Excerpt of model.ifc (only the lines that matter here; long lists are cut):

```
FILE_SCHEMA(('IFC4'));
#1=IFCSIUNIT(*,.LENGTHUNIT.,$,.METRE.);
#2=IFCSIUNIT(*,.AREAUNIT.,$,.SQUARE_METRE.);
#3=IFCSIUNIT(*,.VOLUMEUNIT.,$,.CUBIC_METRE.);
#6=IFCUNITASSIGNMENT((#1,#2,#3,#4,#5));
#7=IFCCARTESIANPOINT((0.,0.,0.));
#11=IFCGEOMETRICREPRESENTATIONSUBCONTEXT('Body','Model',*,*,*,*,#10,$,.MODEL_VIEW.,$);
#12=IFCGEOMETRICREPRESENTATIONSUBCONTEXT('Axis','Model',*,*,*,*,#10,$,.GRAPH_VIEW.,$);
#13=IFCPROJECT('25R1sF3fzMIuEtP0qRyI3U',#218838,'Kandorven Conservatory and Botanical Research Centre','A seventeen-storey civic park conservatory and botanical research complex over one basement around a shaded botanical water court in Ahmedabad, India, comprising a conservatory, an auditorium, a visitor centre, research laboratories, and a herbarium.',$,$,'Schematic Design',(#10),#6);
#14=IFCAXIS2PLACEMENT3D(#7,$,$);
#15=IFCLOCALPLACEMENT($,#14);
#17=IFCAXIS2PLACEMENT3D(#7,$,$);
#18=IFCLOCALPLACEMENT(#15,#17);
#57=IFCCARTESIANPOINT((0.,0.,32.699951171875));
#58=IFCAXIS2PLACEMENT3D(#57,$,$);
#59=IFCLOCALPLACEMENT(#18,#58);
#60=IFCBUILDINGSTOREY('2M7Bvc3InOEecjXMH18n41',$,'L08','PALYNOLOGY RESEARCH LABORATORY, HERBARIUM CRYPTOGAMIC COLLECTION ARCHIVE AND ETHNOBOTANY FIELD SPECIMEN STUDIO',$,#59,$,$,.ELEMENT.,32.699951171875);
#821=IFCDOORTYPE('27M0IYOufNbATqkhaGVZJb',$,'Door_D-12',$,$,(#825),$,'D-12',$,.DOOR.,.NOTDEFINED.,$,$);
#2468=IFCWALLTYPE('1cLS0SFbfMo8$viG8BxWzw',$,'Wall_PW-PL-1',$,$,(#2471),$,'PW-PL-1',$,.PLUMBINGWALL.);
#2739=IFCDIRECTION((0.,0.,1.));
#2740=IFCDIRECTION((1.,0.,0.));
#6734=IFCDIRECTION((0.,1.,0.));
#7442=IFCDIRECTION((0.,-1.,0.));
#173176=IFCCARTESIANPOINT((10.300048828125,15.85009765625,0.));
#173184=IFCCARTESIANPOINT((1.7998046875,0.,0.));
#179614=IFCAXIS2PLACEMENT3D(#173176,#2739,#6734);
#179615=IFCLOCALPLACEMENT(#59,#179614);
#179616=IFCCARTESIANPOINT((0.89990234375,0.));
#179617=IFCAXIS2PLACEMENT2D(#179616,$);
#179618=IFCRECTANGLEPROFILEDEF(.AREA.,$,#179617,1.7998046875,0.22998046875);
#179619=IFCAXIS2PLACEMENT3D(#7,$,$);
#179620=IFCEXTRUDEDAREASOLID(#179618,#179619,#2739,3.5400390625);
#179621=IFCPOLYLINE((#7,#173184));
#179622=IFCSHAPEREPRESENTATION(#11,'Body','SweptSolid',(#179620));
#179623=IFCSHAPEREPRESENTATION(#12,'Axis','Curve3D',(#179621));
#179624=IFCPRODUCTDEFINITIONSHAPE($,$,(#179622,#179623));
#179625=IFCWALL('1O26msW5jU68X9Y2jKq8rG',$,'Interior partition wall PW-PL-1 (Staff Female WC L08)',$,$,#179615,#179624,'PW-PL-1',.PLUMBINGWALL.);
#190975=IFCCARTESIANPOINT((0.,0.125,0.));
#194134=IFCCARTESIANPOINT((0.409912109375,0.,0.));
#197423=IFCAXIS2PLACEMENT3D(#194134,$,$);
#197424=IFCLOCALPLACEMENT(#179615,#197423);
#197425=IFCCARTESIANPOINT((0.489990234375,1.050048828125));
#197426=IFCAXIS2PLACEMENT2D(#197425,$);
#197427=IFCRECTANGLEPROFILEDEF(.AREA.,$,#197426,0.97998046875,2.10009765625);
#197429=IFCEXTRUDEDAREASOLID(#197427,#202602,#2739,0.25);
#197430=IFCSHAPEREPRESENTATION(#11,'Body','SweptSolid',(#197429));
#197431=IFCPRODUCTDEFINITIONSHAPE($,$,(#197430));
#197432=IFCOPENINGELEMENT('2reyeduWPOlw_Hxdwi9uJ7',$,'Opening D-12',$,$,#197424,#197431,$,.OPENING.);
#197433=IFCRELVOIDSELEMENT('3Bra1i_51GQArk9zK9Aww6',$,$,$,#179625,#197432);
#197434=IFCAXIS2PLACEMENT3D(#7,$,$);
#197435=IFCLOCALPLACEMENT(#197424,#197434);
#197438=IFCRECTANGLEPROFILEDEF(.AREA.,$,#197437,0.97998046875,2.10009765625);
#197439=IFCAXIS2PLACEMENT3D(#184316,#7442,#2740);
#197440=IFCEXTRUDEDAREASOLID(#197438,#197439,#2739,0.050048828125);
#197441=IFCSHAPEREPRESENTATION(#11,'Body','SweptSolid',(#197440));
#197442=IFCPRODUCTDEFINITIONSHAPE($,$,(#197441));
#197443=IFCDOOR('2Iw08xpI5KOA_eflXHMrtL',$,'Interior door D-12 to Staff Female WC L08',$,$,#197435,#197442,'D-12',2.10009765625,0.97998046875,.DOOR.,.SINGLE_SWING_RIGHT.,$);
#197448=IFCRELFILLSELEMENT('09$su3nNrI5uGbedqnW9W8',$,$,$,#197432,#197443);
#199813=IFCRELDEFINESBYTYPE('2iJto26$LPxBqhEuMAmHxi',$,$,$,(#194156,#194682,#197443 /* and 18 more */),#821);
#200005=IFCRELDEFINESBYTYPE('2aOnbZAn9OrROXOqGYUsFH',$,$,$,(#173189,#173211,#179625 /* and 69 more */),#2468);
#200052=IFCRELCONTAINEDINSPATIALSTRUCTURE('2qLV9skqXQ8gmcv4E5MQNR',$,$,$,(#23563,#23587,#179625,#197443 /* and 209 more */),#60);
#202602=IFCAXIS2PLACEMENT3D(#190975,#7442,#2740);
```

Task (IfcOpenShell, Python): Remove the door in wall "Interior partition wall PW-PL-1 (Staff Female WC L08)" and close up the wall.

```python
import ifcopenshell
import ifcopenshell.api.feature
import ifcopenshell.api.root
import ifcopenshell.geom
import ifcopenshell.util.shape

model = ifcopenshell.open("model.ifc")
settings = ifcopenshell.geom.settings()


def volume(element):
    """Net volume in cubic metres, openings subtracted."""
    shape = ifcopenshell.geom.create_shape(settings, element)
    return ifcopenshell.util.shape.get_volume(shape.geometry)


door = model.by_guid("2Iw08xpI5KOA_eflXHMrtL")
opening = door.FillsVoids[0].RelatingOpeningElement
wall = opening.VoidsElements[0].RelatingBuildingElement
before = volume(wall)

ifcopenshell.api.root.remove_product(model, product=door)
ifcopenshell.api.feature.remove_feature(model, feature=opening)

after = volume(wall)

print(f"wall volume {before:.3f} -> {after:.3f} m3")

model.write("model_updated.ifc")
```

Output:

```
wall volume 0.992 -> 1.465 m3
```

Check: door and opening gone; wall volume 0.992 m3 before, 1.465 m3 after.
